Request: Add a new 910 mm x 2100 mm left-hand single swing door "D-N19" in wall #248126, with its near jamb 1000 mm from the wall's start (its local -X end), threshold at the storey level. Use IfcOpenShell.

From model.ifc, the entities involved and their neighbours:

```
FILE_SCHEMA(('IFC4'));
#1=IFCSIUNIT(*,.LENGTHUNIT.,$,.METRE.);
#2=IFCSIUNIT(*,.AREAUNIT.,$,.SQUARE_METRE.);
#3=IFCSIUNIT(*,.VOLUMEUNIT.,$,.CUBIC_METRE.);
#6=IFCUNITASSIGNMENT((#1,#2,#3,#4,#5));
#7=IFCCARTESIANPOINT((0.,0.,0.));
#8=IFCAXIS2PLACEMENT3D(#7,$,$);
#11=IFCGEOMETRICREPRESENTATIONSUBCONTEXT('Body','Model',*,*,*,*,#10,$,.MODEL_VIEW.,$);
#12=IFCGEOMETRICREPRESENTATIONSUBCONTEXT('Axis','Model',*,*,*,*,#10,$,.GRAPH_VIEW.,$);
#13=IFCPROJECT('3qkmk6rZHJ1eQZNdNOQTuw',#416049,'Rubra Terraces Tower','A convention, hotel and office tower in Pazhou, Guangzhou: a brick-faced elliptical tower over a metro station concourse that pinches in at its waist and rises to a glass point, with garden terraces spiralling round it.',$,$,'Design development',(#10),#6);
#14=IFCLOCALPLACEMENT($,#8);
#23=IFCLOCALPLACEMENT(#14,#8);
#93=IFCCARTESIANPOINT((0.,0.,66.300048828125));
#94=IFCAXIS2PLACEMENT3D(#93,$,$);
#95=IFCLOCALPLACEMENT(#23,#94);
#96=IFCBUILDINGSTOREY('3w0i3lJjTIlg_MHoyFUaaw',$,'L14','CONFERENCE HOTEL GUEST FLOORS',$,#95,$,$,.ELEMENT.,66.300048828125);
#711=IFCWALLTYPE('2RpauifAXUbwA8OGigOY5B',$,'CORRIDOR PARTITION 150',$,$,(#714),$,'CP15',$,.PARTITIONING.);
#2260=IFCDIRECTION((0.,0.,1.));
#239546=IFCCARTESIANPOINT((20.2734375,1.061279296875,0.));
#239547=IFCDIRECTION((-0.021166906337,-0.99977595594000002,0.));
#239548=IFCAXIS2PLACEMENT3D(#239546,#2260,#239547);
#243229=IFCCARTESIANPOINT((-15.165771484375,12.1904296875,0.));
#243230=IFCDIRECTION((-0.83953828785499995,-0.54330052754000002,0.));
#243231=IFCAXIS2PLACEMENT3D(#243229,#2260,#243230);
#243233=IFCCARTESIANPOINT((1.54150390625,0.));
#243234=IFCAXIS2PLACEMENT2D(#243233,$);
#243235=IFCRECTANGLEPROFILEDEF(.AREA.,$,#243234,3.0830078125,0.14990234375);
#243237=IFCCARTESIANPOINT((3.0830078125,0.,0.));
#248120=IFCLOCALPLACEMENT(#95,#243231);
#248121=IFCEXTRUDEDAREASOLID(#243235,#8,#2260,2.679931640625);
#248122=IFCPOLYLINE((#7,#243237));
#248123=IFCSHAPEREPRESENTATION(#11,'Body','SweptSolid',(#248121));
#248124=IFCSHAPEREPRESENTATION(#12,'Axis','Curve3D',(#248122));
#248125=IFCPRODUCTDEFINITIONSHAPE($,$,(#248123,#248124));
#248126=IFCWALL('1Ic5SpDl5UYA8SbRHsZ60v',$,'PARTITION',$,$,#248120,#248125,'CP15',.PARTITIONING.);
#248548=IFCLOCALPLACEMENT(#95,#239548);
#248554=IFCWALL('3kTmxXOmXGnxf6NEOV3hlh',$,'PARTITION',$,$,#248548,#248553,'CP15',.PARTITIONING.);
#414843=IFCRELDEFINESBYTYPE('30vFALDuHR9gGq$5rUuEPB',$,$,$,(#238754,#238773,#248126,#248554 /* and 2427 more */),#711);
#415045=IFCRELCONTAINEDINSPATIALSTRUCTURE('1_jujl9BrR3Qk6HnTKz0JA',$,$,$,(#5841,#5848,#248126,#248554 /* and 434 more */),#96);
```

```python
import numpy as np
import ifcopenshell
import ifcopenshell.api.feature
import ifcopenshell.api.geometry
import ifcopenshell.api.root
import ifcopenshell.api.spatial
import ifcopenshell.geom
import ifcopenshell.util.element
import ifcopenshell.util.placement
import ifcopenshell.util.representation
import ifcopenshell.util.shape
import ifcopenshell.util.unit

model = ifcopenshell.open("model.ifc")
unit_scale = ifcopenshell.util.unit.calculate_unit_scale(model)
settings = ifcopenshell.geom.settings()


def volume(element):
    """Net volume in cubic metres, openings subtracted."""
    shape = ifcopenshell.geom.create_shape(settings, element)
    return ifcopenshell.util.shape.get_volume(shape.geometry)


wall = model.by_guid("1Ic5SpDl5UYA8SbRHsZ60v")
storey = ifcopenshell.util.element.get_container(wall, ifc_class="IfcBuildingStorey")
context = ifcopenshell.util.representation.get_context(model, "Model", "Body", "MODEL_VIEW")
before = volume(wall)

width, height, from_end, sill = 0.91, 2.1, 1, 0.0  # metres

# The wall runs along its own X axis, and the end named is its -X end.
wall_shape = ifcopenshell.geom.create_shape(settings, wall)
x, y, z = ifcopenshell.util.shape.get_vertices(wall_shape.geometry).T
start = x.min() + from_end
face, thickness = float(y.min()), float(y.max() - y.min())
wall_matrix = ifcopenshell.util.placement.get_local_placement(wall.ObjectPlacement)
level = ifcopenshell.util.placement.get_local_placement(storey.ObjectPlacement)[2, 3]


def in_wall(x, y):
    """Placement at x, y metres in the wall's axes, at sill height."""
    matrix = wall_matrix.copy()
    matrix[:, 3] = wall_matrix @ np.array([x / unit_scale, y / unit_scale, 0.0, 1.0])
    matrix[2, 3] = level + sill / unit_scale
    return matrix


# Opening: a box that overshoots both wall faces by 50 mm.
opening = ifcopenshell.api.root.create_entity(model, ifc_class="IfcOpeningElement", predefined_type="OPENING")
box = ifcopenshell.api.geometry.add_wall_representation(
    model, context=context, length=width, height=height, thickness=thickness + 0.1
)
ifcopenshell.api.geometry.assign_representation(model, product=opening, representation=box)
ifcopenshell.api.geometry.edit_object_placement(model, product=opening, matrix=in_wall(start, face - 0.05), is_si=False)
ifcopenshell.api.feature.add_feature(model, feature=opening, element=wall)

door = ifcopenshell.api.root.create_entity(model, ifc_class="IfcDoor", name="D-N19", predefined_type="DOOR")
door.OverallWidth, door.OverallHeight = width / unit_scale, height / unit_scale
door.OperationType = "SINGLE_SWING_LEFT"
body = ifcopenshell.api.geometry.add_door_representation(
    model,
    context=context,
    overall_width=door.OverallWidth,
    overall_height=door.OverallHeight,
    operation_type="SINGLE_SWING_LEFT",
    lining_properties={"LiningDepth": thickness / unit_scale, "ThresholdDepth": thickness / unit_scale},
)
ifcopenshell.api.geometry.assign_representation(model, product=door, representation=body)
ifcopenshell.api.spatial.assign_container(model, products=[door], relating_structure=storey)
ifcopenshell.api.feature.add_filling(model, opening=opening, element=door)

# The lining spans the wall, so the door starts at the wall face.
ifcopenshell.api.geometry.edit_object_placement(model, product=door, matrix=in_wall(start, face), is_si=False)

after = volume(wall)

print(f"wall volume {before:.3f} -> {after:.3f} m3")

model.write("model_edited.ifc")
```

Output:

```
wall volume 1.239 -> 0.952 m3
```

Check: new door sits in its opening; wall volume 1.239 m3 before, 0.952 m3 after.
